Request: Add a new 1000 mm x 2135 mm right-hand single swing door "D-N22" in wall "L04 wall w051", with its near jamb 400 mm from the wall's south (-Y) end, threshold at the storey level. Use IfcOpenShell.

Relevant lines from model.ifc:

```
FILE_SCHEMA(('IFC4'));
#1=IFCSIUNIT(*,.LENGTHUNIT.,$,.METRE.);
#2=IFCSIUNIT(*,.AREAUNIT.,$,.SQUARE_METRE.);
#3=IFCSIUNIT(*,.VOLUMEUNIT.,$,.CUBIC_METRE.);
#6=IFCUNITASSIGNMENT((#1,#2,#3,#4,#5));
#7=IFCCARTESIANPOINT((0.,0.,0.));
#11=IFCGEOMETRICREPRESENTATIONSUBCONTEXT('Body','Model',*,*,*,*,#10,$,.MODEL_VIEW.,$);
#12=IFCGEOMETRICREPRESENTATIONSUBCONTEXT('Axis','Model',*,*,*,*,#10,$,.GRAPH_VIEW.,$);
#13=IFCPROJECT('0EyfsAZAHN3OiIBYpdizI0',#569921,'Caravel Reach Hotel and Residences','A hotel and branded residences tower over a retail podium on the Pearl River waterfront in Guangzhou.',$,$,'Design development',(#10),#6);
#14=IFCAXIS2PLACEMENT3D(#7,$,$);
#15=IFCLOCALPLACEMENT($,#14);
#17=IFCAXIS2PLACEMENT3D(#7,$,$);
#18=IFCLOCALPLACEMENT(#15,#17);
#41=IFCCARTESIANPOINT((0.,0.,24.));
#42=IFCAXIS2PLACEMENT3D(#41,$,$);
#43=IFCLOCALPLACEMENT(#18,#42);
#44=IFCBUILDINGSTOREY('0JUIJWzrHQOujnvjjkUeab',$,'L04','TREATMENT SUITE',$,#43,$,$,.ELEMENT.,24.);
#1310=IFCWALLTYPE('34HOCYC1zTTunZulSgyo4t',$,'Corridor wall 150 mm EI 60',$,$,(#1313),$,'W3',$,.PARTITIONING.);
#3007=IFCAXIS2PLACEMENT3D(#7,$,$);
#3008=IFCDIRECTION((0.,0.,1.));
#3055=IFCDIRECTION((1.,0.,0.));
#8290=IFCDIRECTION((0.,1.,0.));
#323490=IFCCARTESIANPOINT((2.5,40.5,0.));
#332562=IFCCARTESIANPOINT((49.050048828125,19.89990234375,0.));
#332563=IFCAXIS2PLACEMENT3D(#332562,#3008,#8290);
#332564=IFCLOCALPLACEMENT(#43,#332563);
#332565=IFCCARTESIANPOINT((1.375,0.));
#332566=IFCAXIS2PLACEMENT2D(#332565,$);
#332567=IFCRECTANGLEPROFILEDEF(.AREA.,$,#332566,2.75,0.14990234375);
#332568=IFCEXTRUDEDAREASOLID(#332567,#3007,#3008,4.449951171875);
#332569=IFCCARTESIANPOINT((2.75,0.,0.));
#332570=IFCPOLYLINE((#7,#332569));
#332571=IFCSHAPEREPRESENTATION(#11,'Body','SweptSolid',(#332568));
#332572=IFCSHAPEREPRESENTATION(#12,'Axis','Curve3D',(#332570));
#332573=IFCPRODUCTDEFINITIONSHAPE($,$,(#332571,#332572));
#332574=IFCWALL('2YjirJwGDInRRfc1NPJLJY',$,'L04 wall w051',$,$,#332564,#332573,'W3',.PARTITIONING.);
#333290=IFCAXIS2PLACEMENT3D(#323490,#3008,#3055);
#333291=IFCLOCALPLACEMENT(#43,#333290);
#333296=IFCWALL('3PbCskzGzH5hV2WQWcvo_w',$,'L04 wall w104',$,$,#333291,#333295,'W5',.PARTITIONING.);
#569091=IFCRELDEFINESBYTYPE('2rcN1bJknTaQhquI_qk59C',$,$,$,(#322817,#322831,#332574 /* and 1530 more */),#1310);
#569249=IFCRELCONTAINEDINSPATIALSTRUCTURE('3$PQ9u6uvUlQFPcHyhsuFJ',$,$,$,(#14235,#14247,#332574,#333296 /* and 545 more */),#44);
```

```python
import numpy as np
import ifcopenshell
import ifcopenshell.api.feature
import ifcopenshell.api.geometry
import ifcopenshell.api.root
import ifcopenshell.api.spatial
import ifcopenshell.geom
import ifcopenshell.util.element
import ifcopenshell.util.placement
import ifcopenshell.util.representation
import ifcopenshell.util.shape
import ifcopenshell.util.unit

model = ifcopenshell.open("model.ifc")
unit_scale = ifcopenshell.util.unit.calculate_unit_scale(model)
settings = ifcopenshell.geom.settings()


def volume(element):
    """Net volume in cubic metres, openings subtracted."""
    shape = ifcopenshell.geom.create_shape(settings, element)
    return ifcopenshell.util.shape.get_volume(shape.geometry)


wall = model.by_id(332574)
storey = ifcopenshell.util.element.get_container(wall, ifc_class="IfcBuildingStorey")
context = ifcopenshell.util.representation.get_context(model, "Model", "Body", "MODEL_VIEW")
before = volume(wall)

width, height, from_end, sill = 1, 2.135, 0.4, 0.0  # metres

# The wall runs along its own X axis, and the end named is its -X end.
wall_shape = ifcopenshell.geom.create_shape(settings, wall)
x, y, z = ifcopenshell.util.shape.get_vertices(wall_shape.geometry).T
start = x.min() + from_end
face, thickness = float(y.min()), float(y.max() - y.min())
wall_matrix = ifcopenshell.util.placement.get_local_placement(wall.ObjectPlacement)
level = ifcopenshell.util.placement.get_local_placement(storey.ObjectPlacement)[2, 3]


def in_wall(x, y):
    """Placement at x, y metres in the wall's axes, at sill height."""
    matrix = wall_matrix.copy()
    matrix[:, 3] = wall_matrix @ np.array([x / unit_scale, y / unit_scale, 0.0, 1.0])
    matrix[2, 3] = level + sill / unit_scale
    return matrix


# Opening: a box that overshoots both wall faces by 50 mm.
opening = ifcopenshell.api.root.create_entity(model, ifc_class="IfcOpeningElement", predefined_type="OPENING")
box = ifcopenshell.api.geometry.add_wall_representation(
    model, context=context, length=width, height=height, thickness=thickness + 0.1
)
ifcopenshell.api.geometry.assign_representation(model, product=opening, representation=box)
ifcopenshell.api.geometry.edit_object_placement(model, product=opening, matrix=in_wall(start, face - 0.05), is_si=False)
ifcopenshell.api.feature.add_feature(model, feature=opening, element=wall)

door = ifcopenshell.api.root.create_entity(model, ifc_class="IfcDoor", name="D-N22", predefined_type="DOOR")
door.OverallWidth, door.OverallHeight = width / unit_scale, height / unit_scale
door.OperationType = "SINGLE_SWING_RIGHT"
body = ifcopenshell.api.geometry.add_door_representation(
    model,
    context=context,
    overall_width=door.OverallWidth,
    overall_height=door.OverallHeight,
    operation_type="SINGLE_SWING_RIGHT",
    lining_properties={"LiningDepth": thickness / unit_scale, "ThresholdDepth": thickness / unit_scale},
)
ifcopenshell.api.geometry.assign_representation(model, product=door, representation=body)
ifcopenshell.api.spatial.assign_container(model, products=[door], relating_structure=storey)
ifcopenshell.api.feature.add_filling(model, opening=opening, element=door)

# The lining spans the wall, so the door starts at the wall face.
ifcopenshell.api.geometry.edit_object_placement(model, product=door, matrix=in_wall(start, face), is_si=False)

after = volume(wall)

print(f"wall volume {before:.3f} -> {after:.3f} m3")

model.write("model_edited.ifc")
```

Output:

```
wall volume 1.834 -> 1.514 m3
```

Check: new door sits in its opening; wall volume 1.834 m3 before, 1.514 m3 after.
